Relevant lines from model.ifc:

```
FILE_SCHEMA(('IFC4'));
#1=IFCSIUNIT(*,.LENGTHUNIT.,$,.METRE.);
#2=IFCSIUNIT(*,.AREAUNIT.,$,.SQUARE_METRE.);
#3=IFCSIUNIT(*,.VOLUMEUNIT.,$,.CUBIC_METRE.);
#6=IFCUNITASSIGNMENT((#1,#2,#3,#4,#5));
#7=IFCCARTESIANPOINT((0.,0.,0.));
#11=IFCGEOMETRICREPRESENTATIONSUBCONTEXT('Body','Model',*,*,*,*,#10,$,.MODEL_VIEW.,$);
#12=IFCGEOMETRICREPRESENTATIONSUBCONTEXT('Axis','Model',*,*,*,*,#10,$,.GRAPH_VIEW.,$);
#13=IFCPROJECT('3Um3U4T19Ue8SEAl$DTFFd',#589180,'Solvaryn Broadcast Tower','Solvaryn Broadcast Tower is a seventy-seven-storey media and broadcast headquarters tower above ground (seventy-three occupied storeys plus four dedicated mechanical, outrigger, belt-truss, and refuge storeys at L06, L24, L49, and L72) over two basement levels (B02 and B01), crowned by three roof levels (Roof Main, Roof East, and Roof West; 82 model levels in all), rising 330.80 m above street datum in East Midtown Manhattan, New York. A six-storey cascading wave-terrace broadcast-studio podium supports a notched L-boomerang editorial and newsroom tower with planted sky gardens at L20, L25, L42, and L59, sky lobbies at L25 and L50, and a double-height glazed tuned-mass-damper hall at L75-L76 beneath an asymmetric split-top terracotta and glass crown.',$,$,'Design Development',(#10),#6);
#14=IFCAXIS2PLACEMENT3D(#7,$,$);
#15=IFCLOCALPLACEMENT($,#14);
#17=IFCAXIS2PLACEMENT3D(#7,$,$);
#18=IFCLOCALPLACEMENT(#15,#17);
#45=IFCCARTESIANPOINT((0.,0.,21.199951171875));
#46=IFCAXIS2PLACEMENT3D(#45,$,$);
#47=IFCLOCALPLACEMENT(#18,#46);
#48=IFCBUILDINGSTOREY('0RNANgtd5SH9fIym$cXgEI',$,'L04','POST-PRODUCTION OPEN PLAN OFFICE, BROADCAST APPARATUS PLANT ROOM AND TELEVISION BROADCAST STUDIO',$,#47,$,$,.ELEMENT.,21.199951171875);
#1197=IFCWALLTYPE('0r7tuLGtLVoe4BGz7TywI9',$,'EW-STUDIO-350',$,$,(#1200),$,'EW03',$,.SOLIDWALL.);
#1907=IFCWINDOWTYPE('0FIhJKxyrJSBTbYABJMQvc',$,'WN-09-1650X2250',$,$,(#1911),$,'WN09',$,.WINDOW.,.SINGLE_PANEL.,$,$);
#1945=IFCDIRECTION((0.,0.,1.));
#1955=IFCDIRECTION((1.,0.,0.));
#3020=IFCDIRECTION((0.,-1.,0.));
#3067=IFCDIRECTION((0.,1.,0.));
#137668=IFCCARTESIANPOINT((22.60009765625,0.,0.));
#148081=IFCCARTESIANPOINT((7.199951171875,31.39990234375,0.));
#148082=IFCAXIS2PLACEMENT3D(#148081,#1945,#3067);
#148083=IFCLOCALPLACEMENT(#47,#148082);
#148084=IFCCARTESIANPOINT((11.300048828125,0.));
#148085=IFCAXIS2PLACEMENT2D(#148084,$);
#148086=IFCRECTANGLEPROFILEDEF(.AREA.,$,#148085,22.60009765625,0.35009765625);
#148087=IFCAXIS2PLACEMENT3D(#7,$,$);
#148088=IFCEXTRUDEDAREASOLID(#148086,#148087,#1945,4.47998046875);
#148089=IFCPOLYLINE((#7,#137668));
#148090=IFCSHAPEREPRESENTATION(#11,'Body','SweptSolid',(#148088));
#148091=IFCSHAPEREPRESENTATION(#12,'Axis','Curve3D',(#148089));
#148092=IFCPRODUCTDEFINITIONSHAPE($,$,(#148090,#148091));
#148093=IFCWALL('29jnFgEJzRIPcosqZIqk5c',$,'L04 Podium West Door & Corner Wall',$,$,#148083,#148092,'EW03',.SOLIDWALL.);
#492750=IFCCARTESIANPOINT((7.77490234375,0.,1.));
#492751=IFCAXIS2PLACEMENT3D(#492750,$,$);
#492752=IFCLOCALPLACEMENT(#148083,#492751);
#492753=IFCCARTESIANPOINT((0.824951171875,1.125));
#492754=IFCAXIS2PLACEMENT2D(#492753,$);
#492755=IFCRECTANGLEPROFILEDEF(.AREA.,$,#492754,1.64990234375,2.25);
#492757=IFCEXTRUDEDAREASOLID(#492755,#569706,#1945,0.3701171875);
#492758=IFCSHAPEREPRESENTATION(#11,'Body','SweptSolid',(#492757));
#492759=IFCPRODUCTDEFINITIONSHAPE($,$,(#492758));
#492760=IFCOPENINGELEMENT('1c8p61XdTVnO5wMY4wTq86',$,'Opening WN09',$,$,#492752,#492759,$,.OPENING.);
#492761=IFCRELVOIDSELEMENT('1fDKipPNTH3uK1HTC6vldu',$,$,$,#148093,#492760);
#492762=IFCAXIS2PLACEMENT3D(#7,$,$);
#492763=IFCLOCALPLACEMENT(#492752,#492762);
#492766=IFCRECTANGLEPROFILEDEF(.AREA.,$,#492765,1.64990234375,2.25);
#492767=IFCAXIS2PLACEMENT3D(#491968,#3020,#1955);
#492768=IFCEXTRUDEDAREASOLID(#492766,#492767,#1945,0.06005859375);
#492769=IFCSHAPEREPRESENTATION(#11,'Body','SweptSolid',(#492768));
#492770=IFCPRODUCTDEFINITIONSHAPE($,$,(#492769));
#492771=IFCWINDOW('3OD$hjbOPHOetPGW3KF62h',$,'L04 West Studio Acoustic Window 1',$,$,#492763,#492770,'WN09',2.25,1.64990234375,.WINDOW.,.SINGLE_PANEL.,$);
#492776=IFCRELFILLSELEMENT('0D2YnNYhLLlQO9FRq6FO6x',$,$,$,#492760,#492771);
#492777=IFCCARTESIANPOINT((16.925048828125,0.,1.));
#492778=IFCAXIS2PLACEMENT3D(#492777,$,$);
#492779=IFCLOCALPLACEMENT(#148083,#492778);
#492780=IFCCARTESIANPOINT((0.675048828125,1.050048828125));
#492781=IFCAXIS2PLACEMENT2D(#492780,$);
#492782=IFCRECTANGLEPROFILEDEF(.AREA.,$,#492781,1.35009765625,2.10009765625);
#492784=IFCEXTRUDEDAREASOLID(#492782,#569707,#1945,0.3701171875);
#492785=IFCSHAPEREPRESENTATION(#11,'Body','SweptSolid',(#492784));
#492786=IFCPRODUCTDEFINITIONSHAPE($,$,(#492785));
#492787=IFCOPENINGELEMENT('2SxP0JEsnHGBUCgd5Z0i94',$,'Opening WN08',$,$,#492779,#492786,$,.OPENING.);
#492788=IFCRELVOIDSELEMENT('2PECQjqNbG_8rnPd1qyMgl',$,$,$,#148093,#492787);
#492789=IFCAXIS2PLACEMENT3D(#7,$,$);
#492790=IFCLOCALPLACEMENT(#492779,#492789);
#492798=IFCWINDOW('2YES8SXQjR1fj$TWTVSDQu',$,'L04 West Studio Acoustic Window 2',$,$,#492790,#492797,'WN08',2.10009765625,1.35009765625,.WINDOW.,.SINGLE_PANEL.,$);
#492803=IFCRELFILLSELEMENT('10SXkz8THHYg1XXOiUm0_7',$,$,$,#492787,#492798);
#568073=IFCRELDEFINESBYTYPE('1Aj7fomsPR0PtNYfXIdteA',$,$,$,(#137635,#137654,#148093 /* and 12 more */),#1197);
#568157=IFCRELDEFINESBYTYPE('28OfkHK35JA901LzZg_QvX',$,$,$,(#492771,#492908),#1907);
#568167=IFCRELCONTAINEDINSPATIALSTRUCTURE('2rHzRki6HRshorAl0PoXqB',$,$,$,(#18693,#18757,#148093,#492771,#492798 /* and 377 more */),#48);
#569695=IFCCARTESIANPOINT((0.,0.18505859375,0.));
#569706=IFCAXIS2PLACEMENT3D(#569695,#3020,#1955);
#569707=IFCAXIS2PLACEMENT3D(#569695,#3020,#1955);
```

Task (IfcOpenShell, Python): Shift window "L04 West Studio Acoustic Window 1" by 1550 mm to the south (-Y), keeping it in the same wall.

```python
import ifcopenshell
import ifcopenshell.api.geometry
import ifcopenshell.util.placement
import ifcopenshell.util.unit

model = ifcopenshell.open("model.ifc")
unit_scale = ifcopenshell.util.unit.calculate_unit_scale(model)

window = model.by_guid("3OD$hjbOPHOetPGW3KF62h")
opening = window.FillsVoids[0].RelatingOpeningElement
wall = opening.VoidsElements[0].RelatingBuildingElement

wall_matrix = ifcopenshell.util.placement.get_local_placement(wall.ObjectPlacement)
shift = wall_matrix[:3, 0] * -1.55 / unit_scale
before = ifcopenshell.util.placement.get_local_placement(window.ObjectPlacement)[:3, 3].copy()

# The window is placed relative to its opening, so it follows when the opening moves.
matrix = ifcopenshell.util.placement.get_local_placement(opening.ObjectPlacement)
matrix[:3, 3] += shift
ifcopenshell.api.geometry.edit_object_placement(
    model, product=opening, matrix=matrix, is_si=False, should_transform_children=True
)

after = ifcopenshell.util.placement.get_local_placement(window.ObjectPlacement)[:3, 3]
print("window moved by", (after - before).round(3) + 0.0)

model.write("model_rev.ifc")
```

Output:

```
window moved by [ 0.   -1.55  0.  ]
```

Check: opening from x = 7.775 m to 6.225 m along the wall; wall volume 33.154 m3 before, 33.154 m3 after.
